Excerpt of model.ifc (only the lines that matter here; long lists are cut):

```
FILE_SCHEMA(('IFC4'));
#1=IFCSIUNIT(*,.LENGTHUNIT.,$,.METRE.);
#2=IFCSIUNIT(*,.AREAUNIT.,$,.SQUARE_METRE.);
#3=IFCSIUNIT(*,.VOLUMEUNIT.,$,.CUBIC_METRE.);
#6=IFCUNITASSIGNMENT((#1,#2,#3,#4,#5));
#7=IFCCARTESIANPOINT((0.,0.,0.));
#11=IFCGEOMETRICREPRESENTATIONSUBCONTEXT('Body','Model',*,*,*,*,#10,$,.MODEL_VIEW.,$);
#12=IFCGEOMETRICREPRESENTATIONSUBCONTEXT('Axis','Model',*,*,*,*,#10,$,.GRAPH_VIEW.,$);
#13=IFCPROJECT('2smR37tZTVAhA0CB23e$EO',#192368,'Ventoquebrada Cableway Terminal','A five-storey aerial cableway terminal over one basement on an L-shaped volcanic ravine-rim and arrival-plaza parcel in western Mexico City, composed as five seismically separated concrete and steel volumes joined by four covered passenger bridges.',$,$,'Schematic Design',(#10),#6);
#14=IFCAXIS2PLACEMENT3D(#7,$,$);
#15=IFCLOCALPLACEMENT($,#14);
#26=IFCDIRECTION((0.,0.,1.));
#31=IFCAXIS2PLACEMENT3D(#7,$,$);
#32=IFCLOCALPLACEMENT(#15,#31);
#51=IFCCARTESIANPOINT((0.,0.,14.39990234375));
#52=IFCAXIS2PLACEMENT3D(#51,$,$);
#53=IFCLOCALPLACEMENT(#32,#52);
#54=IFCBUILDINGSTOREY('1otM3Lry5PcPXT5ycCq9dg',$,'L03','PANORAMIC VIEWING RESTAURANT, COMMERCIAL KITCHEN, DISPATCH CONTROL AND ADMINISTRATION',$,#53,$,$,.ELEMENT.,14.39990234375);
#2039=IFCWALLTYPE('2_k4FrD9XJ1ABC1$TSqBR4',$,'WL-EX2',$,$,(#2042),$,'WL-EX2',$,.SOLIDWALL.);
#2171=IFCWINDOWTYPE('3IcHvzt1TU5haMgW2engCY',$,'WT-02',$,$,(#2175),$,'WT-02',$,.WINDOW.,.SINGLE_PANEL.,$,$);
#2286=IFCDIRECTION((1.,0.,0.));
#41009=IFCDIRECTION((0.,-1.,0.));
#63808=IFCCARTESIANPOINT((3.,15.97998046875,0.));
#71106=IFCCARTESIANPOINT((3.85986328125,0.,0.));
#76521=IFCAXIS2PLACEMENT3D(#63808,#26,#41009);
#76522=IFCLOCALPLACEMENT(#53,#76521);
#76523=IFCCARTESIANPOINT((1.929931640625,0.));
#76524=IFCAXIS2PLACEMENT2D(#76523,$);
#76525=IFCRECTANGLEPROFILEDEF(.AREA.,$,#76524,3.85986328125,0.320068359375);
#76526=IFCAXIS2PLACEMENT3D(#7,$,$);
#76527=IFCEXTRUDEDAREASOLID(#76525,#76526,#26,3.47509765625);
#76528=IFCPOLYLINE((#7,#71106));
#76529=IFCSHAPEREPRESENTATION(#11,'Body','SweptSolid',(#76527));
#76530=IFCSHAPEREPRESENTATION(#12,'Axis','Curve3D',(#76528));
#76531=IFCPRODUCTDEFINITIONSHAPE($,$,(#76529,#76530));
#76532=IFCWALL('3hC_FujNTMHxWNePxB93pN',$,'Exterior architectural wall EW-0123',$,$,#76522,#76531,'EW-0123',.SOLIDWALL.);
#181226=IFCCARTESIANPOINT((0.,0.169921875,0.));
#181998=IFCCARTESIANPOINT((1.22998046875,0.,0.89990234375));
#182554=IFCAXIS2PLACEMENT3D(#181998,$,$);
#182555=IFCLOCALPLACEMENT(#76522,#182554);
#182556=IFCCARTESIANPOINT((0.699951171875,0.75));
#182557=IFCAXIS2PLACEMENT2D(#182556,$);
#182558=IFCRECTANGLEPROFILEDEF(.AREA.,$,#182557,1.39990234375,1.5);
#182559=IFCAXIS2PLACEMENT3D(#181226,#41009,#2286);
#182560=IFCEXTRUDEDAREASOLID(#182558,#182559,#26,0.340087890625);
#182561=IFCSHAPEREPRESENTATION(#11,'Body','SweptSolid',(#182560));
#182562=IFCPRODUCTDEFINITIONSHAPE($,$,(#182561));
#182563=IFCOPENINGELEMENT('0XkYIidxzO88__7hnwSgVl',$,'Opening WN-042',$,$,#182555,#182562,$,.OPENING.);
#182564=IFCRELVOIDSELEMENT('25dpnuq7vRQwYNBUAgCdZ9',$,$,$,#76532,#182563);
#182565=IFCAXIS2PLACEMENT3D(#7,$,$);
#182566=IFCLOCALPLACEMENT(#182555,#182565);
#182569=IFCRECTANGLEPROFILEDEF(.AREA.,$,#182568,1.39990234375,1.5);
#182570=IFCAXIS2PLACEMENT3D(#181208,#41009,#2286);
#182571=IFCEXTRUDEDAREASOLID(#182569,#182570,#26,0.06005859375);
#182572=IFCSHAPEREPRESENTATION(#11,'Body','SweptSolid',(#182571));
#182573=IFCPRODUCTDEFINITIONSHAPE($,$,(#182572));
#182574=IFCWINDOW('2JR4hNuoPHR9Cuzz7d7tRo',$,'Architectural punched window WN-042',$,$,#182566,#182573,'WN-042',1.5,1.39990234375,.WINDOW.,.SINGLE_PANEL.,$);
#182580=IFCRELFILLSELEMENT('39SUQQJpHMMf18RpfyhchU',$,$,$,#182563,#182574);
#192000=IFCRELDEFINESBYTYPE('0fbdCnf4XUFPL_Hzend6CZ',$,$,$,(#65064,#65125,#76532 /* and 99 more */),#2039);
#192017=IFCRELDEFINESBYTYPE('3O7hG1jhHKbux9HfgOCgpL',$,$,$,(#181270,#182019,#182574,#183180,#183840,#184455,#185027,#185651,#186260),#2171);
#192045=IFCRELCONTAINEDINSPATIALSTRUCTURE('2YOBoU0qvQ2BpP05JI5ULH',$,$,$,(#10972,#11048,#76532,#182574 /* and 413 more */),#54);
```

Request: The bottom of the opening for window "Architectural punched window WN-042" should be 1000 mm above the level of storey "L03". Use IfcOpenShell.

```python
import numpy as np
import ifcopenshell
import ifcopenshell.api.geometry
import ifcopenshell.geom
import ifcopenshell.util.element
import ifcopenshell.util.placement
import ifcopenshell.util.shape
import ifcopenshell.util.unit

model = ifcopenshell.open("model.ifc")
unit_scale = ifcopenshell.util.unit.calculate_unit_scale(model)

window = model.by_guid("2JR4hNuoPHR9Cuzz7d7tRo")
opening = window.FillsVoids[0].RelatingOpeningElement
storey = ifcopenshell.util.element.get_container(window, ifc_class="IfcBuildingStorey")
level = ifcopenshell.util.placement.get_local_placement(storey.ObjectPlacement)[2, 3]

# The opening's origin need not be at the sill, so measure its lowest point.
shape = ifcopenshell.geom.create_shape(ifcopenshell.geom.settings(), opening)
bottom = ifcopenshell.util.shape.get_shape_bottom_elevation(shape, shape.geometry) / unit_scale
dz = level + 1 / unit_scale - bottom

shift = np.array([0.0, 0.0, dz])
# The window is placed relative to its opening, so it follows when the opening moves.
matrix = ifcopenshell.util.placement.get_local_placement(opening.ObjectPlacement)
matrix[:3, 3] += shift
ifcopenshell.api.geometry.edit_object_placement(
    model, product=opening, matrix=matrix, is_si=False, should_transform_children=True
)

print(f"moved by {dz * unit_scale:+.3f} m")

model.write("model-out.ifc")
```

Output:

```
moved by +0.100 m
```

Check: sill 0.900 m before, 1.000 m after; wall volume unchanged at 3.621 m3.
